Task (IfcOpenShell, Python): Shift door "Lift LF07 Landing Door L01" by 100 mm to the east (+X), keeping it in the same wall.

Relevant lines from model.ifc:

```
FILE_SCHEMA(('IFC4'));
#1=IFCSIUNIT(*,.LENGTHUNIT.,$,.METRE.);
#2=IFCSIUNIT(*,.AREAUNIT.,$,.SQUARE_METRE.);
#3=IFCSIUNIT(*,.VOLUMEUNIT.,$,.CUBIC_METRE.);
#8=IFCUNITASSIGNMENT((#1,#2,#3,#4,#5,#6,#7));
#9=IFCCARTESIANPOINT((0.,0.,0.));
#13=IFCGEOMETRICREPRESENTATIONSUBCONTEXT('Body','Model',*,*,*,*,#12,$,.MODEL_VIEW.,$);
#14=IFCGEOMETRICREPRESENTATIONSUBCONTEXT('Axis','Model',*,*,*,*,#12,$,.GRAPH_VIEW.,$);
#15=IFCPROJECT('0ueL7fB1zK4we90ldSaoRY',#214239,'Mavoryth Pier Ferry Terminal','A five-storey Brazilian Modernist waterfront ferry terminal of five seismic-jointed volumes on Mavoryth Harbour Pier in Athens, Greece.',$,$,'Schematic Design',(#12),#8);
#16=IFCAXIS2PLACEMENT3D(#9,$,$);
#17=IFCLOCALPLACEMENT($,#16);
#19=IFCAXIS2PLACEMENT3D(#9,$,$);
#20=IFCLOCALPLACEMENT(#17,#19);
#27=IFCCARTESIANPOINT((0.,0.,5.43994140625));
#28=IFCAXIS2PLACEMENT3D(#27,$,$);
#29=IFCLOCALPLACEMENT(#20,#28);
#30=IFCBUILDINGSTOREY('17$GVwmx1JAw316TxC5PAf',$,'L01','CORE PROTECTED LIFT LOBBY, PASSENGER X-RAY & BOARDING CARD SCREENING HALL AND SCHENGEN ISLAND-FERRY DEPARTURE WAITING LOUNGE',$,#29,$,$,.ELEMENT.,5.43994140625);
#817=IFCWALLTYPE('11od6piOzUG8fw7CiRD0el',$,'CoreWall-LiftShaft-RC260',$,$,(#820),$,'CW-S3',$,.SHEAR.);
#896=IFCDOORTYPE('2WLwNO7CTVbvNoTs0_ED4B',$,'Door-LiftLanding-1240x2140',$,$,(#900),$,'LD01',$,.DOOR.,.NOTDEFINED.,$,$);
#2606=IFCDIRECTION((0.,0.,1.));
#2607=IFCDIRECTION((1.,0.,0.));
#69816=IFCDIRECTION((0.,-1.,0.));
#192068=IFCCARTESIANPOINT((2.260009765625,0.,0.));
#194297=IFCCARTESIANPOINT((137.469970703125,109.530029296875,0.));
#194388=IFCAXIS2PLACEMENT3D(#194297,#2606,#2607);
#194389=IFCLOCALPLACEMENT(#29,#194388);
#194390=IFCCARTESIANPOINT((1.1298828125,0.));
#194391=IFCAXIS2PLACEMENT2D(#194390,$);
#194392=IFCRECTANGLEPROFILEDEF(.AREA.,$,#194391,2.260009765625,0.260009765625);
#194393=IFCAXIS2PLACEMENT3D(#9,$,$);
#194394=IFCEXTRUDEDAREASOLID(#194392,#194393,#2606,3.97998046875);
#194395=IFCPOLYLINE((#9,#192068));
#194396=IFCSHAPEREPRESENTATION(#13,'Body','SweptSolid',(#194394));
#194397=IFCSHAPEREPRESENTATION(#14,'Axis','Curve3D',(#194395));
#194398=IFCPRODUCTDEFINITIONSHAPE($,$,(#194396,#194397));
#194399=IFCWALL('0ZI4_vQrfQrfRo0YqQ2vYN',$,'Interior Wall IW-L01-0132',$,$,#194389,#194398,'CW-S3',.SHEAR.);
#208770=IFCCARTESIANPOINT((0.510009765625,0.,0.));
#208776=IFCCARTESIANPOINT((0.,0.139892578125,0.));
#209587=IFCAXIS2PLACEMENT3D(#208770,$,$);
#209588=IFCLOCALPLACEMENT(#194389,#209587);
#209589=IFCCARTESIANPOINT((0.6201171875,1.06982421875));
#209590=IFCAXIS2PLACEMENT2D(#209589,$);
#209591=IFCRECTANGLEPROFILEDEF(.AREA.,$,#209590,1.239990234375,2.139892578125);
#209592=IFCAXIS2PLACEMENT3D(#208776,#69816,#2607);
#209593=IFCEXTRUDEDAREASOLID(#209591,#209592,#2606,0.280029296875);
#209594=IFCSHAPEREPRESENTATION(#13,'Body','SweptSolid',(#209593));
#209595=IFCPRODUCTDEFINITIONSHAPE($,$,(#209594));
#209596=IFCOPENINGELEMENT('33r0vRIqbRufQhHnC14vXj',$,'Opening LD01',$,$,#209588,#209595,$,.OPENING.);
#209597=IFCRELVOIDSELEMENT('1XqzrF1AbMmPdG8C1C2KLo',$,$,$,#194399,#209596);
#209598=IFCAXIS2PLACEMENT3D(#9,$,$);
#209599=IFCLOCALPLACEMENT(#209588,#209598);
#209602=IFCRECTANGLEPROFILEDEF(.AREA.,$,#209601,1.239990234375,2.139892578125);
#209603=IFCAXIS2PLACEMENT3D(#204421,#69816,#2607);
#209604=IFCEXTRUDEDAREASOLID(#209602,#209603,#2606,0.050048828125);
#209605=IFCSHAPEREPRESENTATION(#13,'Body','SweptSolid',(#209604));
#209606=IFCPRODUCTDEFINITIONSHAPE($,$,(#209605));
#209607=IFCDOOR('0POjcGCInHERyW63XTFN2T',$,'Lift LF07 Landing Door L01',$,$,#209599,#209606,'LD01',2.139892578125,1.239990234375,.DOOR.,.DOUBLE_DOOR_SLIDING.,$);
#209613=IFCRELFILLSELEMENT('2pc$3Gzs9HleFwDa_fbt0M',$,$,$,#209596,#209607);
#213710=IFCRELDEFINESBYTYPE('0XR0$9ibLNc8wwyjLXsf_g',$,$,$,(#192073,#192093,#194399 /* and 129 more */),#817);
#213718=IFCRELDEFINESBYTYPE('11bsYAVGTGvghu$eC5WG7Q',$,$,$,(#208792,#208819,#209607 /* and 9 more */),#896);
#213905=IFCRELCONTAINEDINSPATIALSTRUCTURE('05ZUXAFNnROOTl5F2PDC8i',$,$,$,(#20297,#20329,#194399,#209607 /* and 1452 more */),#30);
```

```python
import ifcopenshell
import ifcopenshell.api.geometry
import ifcopenshell.util.placement
import ifcopenshell.util.unit

model = ifcopenshell.open("model.ifc")
unit_scale = ifcopenshell.util.unit.calculate_unit_scale(model)

door = model.by_guid("0POjcGCInHERyW63XTFN2T")
opening = door.FillsVoids[0].RelatingOpeningElement
wall = opening.VoidsElements[0].RelatingBuildingElement

wall_matrix = ifcopenshell.util.placement.get_local_placement(wall.ObjectPlacement)
shift = wall_matrix[:3, 0] * 0.1 / unit_scale
before = ifcopenshell.util.placement.get_local_placement(door.ObjectPlacement)[:3, 3].copy()

# The door is placed relative to its opening, so it follows when the opening moves.
matrix = ifcopenshell.util.placement.get_local_placement(opening.ObjectPlacement)
matrix[:3, 3] += shift
ifcopenshell.api.geometry.edit_object_placement(
    model, product=opening, matrix=matrix, is_si=False, should_transform_children=True
)

after = ifcopenshell.util.placement.get_local_placement(door.ObjectPlacement)[:3, 3]
print("door moved by", (after - before).round(3) + 0.0)

model.write("model-out.ifc")
```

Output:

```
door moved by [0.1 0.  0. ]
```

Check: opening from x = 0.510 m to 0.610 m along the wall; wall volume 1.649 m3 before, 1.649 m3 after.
